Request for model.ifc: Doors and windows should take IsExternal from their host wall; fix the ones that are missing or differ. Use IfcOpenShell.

First a look at what the model holds.

```python
import ifcopenshell
import ifcopenshell.util.element

model = ifcopenshell.open("model.ifc")
print(model.schema)
seen = {}
for e in model.by_type("IfcDoor") + model.by_type("IfcWindow"):
    if not e.FillsVoids:
        continue
    host = e.FillsVoids[0].RelatingOpeningElement.VoidsElements[0].RelatingBuildingElement
    own = ifcopenshell.util.element.get_pset(e, f"Pset_{e.is_a()[3:].removesuffix('StandardCase')}Common", "IsExternal")
    wall = ifcopenshell.util.element.get_pset(host, "Pset_WallCommon", "IsExternal")
    seen[e.is_a(), own, wall] = seen.get((e.is_a(), own, wall), 0) + 1
for (cls, own, wall), count in sorted(seen.items(), key=str):
    print(count, cls, "IsExternal:", own, "| host wall:", wall)
```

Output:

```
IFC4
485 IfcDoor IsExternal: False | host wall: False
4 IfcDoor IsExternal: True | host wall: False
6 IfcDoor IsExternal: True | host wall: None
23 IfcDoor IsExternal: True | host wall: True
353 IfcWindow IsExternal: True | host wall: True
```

```python
import ifcopenshell
import ifcopenshell.api.pset
import ifcopenshell.util.element

model = ifcopenshell.open("model.ifc")

count = 0
for ifc_class, pset_name in (("IfcDoor", "Pset_DoorCommon"), ("IfcWindow", "Pset_WindowCommon")):
    for e in model.by_type(ifc_class):
        if not e.FillsVoids:
            continue
        host = e.FillsVoids[0].RelatingOpeningElement.VoidsElements[0].RelatingBuildingElement
        external = ifcopenshell.util.element.get_pset(host, "Pset_WallCommon", "IsExternal")
        if external is None or ifcopenshell.util.element.get_pset(e, pset_name, "IsExternal") == external:
            continue
        pset = ifcopenshell.api.pset.add_pset(model, product=e, name=pset_name)
        ifcopenshell.api.pset.edit_pset(model, pset=pset, properties={"IsExternal": external})
        count += 1

print(count, "updated")

model.write("model_edited.ifc")
```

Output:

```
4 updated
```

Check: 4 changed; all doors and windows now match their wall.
